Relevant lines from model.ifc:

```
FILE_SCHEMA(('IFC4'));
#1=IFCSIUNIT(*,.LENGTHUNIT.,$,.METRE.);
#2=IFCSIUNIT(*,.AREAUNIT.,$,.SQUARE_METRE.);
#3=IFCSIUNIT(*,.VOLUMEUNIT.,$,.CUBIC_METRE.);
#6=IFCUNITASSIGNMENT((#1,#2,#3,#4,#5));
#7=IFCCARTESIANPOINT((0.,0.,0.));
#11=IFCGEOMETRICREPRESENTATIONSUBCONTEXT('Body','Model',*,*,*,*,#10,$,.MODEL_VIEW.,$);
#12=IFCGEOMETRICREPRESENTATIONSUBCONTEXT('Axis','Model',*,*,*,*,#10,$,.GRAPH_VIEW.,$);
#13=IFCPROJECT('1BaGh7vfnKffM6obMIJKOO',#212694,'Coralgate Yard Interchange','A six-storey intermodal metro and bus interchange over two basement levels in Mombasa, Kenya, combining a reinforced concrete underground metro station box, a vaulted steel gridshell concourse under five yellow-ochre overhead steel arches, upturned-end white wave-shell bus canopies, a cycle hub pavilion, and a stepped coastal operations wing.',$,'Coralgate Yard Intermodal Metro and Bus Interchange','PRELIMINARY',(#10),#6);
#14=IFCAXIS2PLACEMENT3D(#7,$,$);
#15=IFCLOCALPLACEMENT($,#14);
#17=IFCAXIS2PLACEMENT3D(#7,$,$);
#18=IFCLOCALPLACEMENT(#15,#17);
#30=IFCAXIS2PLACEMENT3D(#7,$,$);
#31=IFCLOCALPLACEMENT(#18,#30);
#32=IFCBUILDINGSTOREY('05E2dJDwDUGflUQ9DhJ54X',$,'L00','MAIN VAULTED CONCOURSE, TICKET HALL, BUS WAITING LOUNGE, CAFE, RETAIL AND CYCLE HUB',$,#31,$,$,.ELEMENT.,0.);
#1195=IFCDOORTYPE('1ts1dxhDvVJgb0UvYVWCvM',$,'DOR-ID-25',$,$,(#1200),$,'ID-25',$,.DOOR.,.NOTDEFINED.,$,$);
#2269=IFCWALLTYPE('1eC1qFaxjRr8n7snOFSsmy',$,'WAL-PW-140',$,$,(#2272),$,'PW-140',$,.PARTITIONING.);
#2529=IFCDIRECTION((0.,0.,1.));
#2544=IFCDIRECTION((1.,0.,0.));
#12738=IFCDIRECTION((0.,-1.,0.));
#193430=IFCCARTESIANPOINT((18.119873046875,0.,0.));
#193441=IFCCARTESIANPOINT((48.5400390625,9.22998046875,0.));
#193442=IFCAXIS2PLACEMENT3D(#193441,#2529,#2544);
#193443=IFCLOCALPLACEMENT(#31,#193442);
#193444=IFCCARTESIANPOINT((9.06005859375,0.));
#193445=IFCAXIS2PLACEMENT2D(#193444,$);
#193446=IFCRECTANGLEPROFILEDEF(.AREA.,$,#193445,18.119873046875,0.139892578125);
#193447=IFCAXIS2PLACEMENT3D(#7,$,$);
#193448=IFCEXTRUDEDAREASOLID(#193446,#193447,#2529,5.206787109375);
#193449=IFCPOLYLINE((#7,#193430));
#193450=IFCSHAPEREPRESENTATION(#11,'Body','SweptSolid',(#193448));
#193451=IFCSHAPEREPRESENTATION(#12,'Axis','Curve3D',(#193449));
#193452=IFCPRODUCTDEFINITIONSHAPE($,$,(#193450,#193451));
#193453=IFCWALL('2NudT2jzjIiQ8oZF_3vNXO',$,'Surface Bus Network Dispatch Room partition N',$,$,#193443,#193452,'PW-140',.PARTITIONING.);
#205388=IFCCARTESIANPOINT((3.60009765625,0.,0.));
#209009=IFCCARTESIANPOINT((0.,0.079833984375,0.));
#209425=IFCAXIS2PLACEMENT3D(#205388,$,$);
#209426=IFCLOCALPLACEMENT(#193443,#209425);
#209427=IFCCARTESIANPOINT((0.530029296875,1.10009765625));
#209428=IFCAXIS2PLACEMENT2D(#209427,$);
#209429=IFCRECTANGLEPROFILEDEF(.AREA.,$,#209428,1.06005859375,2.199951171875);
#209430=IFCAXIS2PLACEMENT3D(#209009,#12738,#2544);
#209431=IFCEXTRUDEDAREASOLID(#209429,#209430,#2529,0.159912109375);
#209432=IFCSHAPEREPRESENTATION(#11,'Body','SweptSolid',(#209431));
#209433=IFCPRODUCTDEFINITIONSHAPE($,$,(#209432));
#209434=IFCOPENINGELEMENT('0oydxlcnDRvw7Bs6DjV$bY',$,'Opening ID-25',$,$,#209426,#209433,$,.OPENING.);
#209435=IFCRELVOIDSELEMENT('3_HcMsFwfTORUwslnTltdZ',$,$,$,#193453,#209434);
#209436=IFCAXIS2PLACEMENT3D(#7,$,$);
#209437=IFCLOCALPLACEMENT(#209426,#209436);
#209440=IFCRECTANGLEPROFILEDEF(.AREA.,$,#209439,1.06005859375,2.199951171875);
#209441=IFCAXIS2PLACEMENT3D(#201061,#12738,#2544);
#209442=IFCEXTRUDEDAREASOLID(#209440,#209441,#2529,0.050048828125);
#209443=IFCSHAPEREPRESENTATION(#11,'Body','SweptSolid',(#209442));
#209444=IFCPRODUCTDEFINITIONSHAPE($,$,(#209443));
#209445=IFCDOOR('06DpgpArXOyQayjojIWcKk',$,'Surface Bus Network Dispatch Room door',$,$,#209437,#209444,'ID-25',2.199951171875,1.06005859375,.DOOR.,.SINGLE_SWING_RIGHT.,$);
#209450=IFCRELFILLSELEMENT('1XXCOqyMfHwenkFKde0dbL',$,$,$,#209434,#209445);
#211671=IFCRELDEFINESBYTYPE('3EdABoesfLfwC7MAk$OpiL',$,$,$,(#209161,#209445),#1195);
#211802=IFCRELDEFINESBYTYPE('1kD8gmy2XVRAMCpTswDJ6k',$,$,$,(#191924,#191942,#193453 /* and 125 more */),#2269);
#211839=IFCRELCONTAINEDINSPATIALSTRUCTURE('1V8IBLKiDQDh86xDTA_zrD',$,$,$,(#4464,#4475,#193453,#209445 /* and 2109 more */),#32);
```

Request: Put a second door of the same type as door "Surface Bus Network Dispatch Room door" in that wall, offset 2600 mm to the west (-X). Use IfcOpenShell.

```python
import ifcopenshell
import ifcopenshell.api.feature
import ifcopenshell.api.geometry
import ifcopenshell.api.root
import ifcopenshell.geom
import ifcopenshell.util.element
import ifcopenshell.util.placement
import ifcopenshell.util.shape
import ifcopenshell.util.unit

model = ifcopenshell.open("model.ifc")
unit_scale = ifcopenshell.util.unit.calculate_unit_scale(model)
settings = ifcopenshell.geom.settings()


def volume(element):
    """Net volume in cubic metres, openings subtracted."""
    shape = ifcopenshell.geom.create_shape(settings, element)
    return ifcopenshell.util.shape.get_volume(shape.geometry)


door = model.by_guid("06DpgpArXOyQayjojIWcKk")
opening = door.FillsVoids[0].RelatingOpeningElement
wall = opening.VoidsElements[0].RelatingBuildingElement
before = volume(wall)
shift = ifcopenshell.util.placement.get_local_placement(wall.ObjectPlacement)[:3, 0] * -2.6 / unit_scale

# copy_class copies the void relationship, type, container and properties, but no geometry.
new_opening = ifcopenshell.api.root.copy_class(model, product=opening)
new_opening.Representation = ifcopenshell.util.element.copy_deep(
    model, opening.Representation, exclude=["IfcGeometricRepresentationContext", "IfcRepresentationMap"]
)
new_door = ifcopenshell.api.root.copy_class(model, product=door)
new_door.Representation = ifcopenshell.util.element.copy_deep(
    model, door.Representation, exclude=["IfcGeometricRepresentationContext", "IfcRepresentationMap"]
)
new_door.Tag = None
ifcopenshell.api.feature.add_filling(model, opening=new_opening, element=new_door)

for old, new in ((opening, new_opening), (door, new_door)):
    matrix = ifcopenshell.util.placement.get_local_placement(old.ObjectPlacement)
    matrix[:3, 3] += shift
    ifcopenshell.api.geometry.edit_object_placement(model, product=new, matrix=matrix, is_si=False)

after = volume(wall)

print(f"wall volume {before:.3f} -> {after:.3f} m3")

model.write("model_edited.ifc")
```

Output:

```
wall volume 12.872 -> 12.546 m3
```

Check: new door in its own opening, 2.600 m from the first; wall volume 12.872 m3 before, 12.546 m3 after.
